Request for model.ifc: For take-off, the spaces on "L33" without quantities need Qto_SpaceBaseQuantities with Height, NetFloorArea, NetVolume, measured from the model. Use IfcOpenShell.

First a look at what the model holds.

```python
import ifcopenshell
import ifcopenshell.util.element
import ifcopenshell.util.unit

model = ifcopenshell.open("model.ifc")
print(model.schema)
for unit_type in ("LENGTHUNIT", "AREAUNIT", "VOLUMEUNIT"):
    print(unit_type, ifcopenshell.util.unit.calculate_unit_scale(model, unit_type))
storey = next(s for s in model.by_type("IfcBuildingStorey") if s.Name == "L33")
spaces = [e for e in ifcopenshell.util.element.get_decomposition(storey) if e.is_a("IfcSpace")]
for e in sorted(spaces, key=lambda e: e.id()):
    print(e.id(), e.is_a(), e.Name, list(ifcopenshell.util.element.get_psets(e, qtos_only=True)), sep=" | ")
```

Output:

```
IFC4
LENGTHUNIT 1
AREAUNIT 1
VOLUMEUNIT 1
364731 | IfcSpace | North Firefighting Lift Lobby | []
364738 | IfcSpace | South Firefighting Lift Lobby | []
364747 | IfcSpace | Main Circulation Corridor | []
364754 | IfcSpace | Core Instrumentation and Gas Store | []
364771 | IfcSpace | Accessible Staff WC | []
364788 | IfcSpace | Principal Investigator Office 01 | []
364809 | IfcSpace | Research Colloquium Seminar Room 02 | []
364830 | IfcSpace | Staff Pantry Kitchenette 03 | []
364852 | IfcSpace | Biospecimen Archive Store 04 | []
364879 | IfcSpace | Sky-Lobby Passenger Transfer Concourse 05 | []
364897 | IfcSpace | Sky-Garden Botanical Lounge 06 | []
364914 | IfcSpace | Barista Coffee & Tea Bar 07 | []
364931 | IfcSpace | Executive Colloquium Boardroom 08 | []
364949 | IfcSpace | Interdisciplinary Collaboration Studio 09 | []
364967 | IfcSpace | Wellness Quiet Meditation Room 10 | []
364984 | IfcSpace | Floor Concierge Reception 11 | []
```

```python
import ifcopenshell
import ifcopenshell.api.pset
import ifcopenshell.geom
import ifcopenshell.util.element
import ifcopenshell.util.shape
import ifcopenshell.util.unit

model = ifcopenshell.open("model.ifc")
unit_scale = ifcopenshell.util.unit.calculate_unit_scale(model)
area_scale = ifcopenshell.util.unit.calculate_unit_scale(model, "AREAUNIT")
volume_scale = ifcopenshell.util.unit.calculate_unit_scale(model, "VOLUMEUNIT")
settings = ifcopenshell.geom.settings()

storey = next(s for s in model.by_type("IfcBuildingStorey") if s.Name == "L33")
spaces = [e for e in ifcopenshell.util.element.get_decomposition(storey) if e.is_a("IfcSpace")]

for e in sorted(spaces, key=lambda e: e.id()):
    if ifcopenshell.util.element.get_psets(e, qtos_only=True, should_inherit=False):
        continue
    # Geometry comes back in metres, in the element's own axes.
    shape = ifcopenshell.geom.create_shape(settings, e)
    values = {
        "Height": ifcopenshell.util.shape.get_z(shape.geometry) / unit_scale,
        "NetFloorArea": ifcopenshell.util.shape.get_footprint_area(shape.geometry) / area_scale,
        "NetVolume": ifcopenshell.util.shape.get_volume(shape.geometry) / volume_scale,
    }
    qto = ifcopenshell.api.pset.add_qto(model, product=e, name="Qto_SpaceBaseQuantities")
    ifcopenshell.api.pset.edit_qto(model, qto=qto, properties=values)
    print(e.id(), {k: round(v, 3) for k, v in values.items()})

model.write("model_updated.ifc")
```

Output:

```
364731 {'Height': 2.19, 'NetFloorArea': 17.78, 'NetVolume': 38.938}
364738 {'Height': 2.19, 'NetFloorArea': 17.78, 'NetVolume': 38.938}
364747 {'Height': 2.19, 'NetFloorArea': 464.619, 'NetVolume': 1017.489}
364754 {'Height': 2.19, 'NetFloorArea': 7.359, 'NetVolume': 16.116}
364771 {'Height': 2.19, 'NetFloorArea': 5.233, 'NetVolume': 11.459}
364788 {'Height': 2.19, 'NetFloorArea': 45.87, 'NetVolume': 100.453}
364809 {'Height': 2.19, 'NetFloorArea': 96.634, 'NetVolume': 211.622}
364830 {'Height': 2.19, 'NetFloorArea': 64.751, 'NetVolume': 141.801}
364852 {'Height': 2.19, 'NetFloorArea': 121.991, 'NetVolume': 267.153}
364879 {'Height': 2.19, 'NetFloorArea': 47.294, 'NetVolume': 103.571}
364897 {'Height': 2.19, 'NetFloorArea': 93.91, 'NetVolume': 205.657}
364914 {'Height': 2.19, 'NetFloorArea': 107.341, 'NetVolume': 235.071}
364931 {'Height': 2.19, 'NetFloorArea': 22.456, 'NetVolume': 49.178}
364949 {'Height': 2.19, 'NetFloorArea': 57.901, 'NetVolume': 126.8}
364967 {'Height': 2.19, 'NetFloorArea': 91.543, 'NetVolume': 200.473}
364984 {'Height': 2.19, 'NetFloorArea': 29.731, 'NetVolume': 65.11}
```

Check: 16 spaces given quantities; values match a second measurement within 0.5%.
